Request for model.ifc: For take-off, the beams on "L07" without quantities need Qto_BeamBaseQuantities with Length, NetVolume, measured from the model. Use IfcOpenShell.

First a look at what the model holds.

```python
import ifcopenshell
import ifcopenshell.util.element
import ifcopenshell.util.unit

model = ifcopenshell.open("model.ifc")
print(model.schema)
for unit_type in ("LENGTHUNIT", "AREAUNIT", "VOLUMEUNIT"):
    print(unit_type, ifcopenshell.util.unit.calculate_unit_scale(model, unit_type))
storey = next(s for s in model.by_type("IfcBuildingStorey") if s.Name == "L07")
beams = [e for e in ifcopenshell.util.element.get_decomposition(storey) if e.is_a("IfcBeam")]
for e in sorted(beams, key=lambda e: e.id()):
    print(e.id(), e.is_a(), e.Name, list(ifcopenshell.util.element.get_psets(e, qtos_only=True)), sep=" | ")
```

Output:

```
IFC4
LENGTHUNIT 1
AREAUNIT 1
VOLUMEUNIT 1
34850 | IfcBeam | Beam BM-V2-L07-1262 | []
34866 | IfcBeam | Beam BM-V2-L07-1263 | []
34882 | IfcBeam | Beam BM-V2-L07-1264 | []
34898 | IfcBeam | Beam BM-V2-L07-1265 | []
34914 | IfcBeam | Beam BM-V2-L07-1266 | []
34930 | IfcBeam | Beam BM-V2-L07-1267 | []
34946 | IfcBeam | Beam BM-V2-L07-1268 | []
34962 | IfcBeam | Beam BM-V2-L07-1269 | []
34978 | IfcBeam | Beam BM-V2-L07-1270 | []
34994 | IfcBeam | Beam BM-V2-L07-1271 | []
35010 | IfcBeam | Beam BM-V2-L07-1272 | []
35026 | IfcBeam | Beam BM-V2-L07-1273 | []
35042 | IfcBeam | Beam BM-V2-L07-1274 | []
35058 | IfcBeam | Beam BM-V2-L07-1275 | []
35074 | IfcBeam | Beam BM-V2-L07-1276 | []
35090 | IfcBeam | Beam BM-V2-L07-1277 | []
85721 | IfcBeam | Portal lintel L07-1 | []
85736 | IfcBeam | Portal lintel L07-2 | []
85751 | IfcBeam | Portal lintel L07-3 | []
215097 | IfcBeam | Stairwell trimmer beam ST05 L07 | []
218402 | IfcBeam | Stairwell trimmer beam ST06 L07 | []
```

```python
import ifcopenshell
import ifcopenshell.api.pset
import ifcopenshell.geom
import ifcopenshell.util.element
import ifcopenshell.util.shape
import ifcopenshell.util.unit

model = ifcopenshell.open("model.ifc")
unit_scale = ifcopenshell.util.unit.calculate_unit_scale(model)
volume_scale = ifcopenshell.util.unit.calculate_unit_scale(model, "VOLUMEUNIT")
settings = ifcopenshell.geom.settings()

storey = next(s for s in model.by_type("IfcBuildingStorey") if s.Name == "L07")
beams = [e for e in ifcopenshell.util.element.get_decomposition(storey) if e.is_a("IfcBeam")]

for e in sorted(beams, key=lambda e: e.id()):
    if ifcopenshell.util.element.get_psets(e, qtos_only=True, should_inherit=False):
        continue
    # Geometry comes back in metres, in the element's own axes.
    shape = ifcopenshell.geom.create_shape(settings, e)
    values = {
        "Length": ifcopenshell.util.shape.get_max_xyz(shape.geometry) / unit_scale,
        "NetVolume": ifcopenshell.util.shape.get_volume(shape.geometry) / volume_scale,
    }
    qto = ifcopenshell.api.pset.add_qto(model, product=e, name="Qto_BeamBaseQuantities")
    ifcopenshell.api.pset.edit_qto(model, qto=qto, properties=values)
    print(e.id(), {k: round(v, 3) for k, v in values.items()})

model.write("model_edited.ifc")
```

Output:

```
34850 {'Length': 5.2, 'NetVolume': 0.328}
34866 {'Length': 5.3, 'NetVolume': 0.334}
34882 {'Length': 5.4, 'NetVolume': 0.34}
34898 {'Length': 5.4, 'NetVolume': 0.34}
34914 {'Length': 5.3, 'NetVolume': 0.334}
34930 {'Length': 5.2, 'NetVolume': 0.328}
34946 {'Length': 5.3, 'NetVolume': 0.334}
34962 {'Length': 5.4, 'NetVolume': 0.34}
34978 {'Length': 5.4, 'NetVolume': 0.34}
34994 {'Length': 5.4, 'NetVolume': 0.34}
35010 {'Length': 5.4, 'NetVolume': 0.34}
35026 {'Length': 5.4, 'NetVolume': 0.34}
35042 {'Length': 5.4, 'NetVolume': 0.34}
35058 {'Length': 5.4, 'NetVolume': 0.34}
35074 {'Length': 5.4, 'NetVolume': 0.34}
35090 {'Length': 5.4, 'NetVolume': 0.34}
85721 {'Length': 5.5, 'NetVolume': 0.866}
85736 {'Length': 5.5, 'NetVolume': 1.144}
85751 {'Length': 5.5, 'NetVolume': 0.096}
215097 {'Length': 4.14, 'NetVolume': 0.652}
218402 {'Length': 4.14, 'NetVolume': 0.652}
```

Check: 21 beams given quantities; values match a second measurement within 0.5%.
